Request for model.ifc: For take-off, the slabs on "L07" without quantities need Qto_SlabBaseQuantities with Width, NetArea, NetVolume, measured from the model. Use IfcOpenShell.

First a look at what the model holds.

```python
import ifcopenshell
import ifcopenshell.util.element
import ifcopenshell.util.unit

model = ifcopenshell.open("model.ifc")
print(model.schema)
for unit_type in ("LENGTHUNIT", "AREAUNIT", "VOLUMEUNIT"):
    print(unit_type, ifcopenshell.util.unit.calculate_unit_scale(model, unit_type))
storey = next(s for s in model.by_type("IfcBuildingStorey") if s.Name == "L07")
slabs = [e for e in ifcopenshell.util.element.get_decomposition(storey) if e.is_a("IfcSlab")]
for e in sorted(slabs, key=lambda e: e.id()):
    print(e.id(), e.is_a(), e.Name, list(ifcopenshell.util.element.get_psets(e, qtos_only=True)), sep=" | ")
```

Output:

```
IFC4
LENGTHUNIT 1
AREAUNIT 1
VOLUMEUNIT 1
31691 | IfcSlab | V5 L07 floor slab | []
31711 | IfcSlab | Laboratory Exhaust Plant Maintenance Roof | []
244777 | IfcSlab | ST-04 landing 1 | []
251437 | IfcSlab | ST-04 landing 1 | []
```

```python
import ifcopenshell
import ifcopenshell.api.pset
import ifcopenshell.geom
import ifcopenshell.util.element
import ifcopenshell.util.shape
import ifcopenshell.util.unit

model = ifcopenshell.open("model.ifc")
unit_scale = ifcopenshell.util.unit.calculate_unit_scale(model)
area_scale = ifcopenshell.util.unit.calculate_unit_scale(model, "AREAUNIT")
volume_scale = ifcopenshell.util.unit.calculate_unit_scale(model, "VOLUMEUNIT")
settings = ifcopenshell.geom.settings()

storey = next(s for s in model.by_type("IfcBuildingStorey") if s.Name == "L07")
slabs = [e for e in ifcopenshell.util.element.get_decomposition(storey) if e.is_a("IfcSlab")]

for e in sorted(slabs, key=lambda e: e.id()):
    if ifcopenshell.util.element.get_psets(e, qtos_only=True, should_inherit=False):
        continue
    # Geometry comes back in metres, in the element's own axes.
    shape = ifcopenshell.geom.create_shape(settings, e)
    values = {
        "Width": ifcopenshell.util.shape.get_z(shape.geometry) / unit_scale,
        "NetArea": ifcopenshell.util.shape.get_footprint_area(shape.geometry) / area_scale,
        "NetVolume": ifcopenshell.util.shape.get_volume(shape.geometry) / volume_scale,
    }
    qto = ifcopenshell.api.pset.add_qto(model, product=e, name="Qto_SlabBaseQuantities")
    ifcopenshell.api.pset.edit_qto(model, qto=qto, properties=values)
    print(e.id(), {k: round(v, 3) for k, v in values.items()})

model.write("model_rev.ifc")
```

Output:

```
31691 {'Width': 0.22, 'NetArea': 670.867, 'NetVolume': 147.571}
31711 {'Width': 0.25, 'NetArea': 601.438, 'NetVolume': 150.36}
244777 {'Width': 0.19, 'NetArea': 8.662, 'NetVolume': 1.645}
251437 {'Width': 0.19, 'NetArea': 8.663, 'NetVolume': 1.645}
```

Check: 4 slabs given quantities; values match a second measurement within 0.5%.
